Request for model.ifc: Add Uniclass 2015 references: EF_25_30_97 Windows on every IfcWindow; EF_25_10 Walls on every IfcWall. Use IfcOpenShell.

First a look at what the model holds.

```python
import ifcopenshell

model = ifcopenshell.open("model.ifc")
print(model.schema)
print("classifications:", [c.Name for c in model.by_type("IfcClassification")])
for ifc_class in ("IfcDoor", "IfcRoof", "IfcStair", "IfcWall", "IfcWindow"):
    print(ifc_class, len(model.by_type(ifc_class)))
```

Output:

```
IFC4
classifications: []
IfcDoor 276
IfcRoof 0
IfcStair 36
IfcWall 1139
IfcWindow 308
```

```python
import ifcopenshell
import ifcopenshell.api.classification

model = ifcopenshell.open("model.ifc")

system = ifcopenshell.api.classification.add_classification(model, classification="Uniclass 2015")

codes = {
    "IfcWindow": ("EF_25_30_97", "Windows"),
    "IfcWall": ("EF_25_10", "Walls"),
}
for ifc_class, (code, name) in codes.items():
    products = model.by_type(ifc_class)
    ifcopenshell.api.classification.add_reference(
        model, products=products, classification=system, identification=code, name=name
    )
    print(code, len(products))

model.write("model-out.ifc")
```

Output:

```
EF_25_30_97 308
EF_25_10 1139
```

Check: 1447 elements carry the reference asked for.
